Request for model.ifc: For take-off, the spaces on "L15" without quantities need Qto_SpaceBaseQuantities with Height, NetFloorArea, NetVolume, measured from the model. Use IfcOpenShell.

First a look at what the model holds.

```python
import ifcopenshell
import ifcopenshell.util.element
import ifcopenshell.util.unit

model = ifcopenshell.open("model.ifc")
print(model.schema)
for unit_type in ("LENGTHUNIT", "AREAUNIT", "VOLUMEUNIT"):
    print(unit_type, ifcopenshell.util.unit.calculate_unit_scale(model, unit_type))
storey = next(s for s in model.by_type("IfcBuildingStorey") if s.Name == "L15")
spaces = [e for e in ifcopenshell.util.element.get_decomposition(storey) if e.is_a("IfcSpace")]
for e in sorted(spaces, key=lambda e: e.id()):
    print(e.id(), e.is_a(), e.Name, list(ifcopenshell.util.element.get_psets(e, qtos_only=True)), sep=" | ")
```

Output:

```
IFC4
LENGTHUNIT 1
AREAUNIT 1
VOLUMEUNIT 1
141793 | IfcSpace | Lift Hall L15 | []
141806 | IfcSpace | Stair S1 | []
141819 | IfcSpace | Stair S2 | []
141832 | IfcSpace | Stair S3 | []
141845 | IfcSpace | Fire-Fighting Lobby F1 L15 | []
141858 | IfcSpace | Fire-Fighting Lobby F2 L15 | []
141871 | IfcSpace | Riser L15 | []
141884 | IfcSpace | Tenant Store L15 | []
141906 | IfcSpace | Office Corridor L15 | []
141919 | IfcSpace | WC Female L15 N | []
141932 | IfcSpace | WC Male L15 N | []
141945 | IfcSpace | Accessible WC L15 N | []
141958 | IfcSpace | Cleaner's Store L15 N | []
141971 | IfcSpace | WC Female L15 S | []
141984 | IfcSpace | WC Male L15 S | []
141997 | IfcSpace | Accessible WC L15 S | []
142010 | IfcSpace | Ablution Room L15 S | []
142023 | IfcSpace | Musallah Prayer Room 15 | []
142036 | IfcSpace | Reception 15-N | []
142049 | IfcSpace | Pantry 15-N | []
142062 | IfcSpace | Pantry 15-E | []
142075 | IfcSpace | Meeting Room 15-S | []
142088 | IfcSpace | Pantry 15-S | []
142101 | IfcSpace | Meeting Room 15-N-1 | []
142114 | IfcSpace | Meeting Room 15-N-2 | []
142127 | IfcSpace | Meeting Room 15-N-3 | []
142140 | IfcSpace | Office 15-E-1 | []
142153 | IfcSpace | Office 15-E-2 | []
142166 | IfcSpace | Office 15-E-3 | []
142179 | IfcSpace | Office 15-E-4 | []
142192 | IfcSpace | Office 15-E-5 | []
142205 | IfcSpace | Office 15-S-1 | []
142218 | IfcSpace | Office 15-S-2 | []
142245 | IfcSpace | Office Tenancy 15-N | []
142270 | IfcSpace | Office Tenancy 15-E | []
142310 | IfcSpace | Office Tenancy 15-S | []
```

```python
import ifcopenshell
import ifcopenshell.api.pset
import ifcopenshell.geom
import ifcopenshell.util.element
import ifcopenshell.util.shape
import ifcopenshell.util.unit

model = ifcopenshell.open("model.ifc")
unit_scale = ifcopenshell.util.unit.calculate_unit_scale(model)
area_scale = ifcopenshell.util.unit.calculate_unit_scale(model, "AREAUNIT")
volume_scale = ifcopenshell.util.unit.calculate_unit_scale(model, "VOLUMEUNIT")
settings = ifcopenshell.geom.settings()

storey = next(s for s in model.by_type("IfcBuildingStorey") if s.Name == "L15")
spaces = [e for e in ifcopenshell.util.element.get_decomposition(storey) if e.is_a("IfcSpace")]

for e in sorted(spaces, key=lambda e: e.id()):
    if ifcopenshell.util.element.get_psets(e, qtos_only=True, should_inherit=False):
        continue
    # Geometry comes back in metres, in the element's own axes.
    shape = ifcopenshell.geom.create_shape(settings, e)
    values = {
        "Height": ifcopenshell.util.shape.get_z(shape.geometry) / unit_scale,
        "NetFloorArea": ifcopenshell.util.shape.get_footprint_area(shape.geometry) / area_scale,
        "NetVolume": ifcopenshell.util.shape.get_volume(shape.geometry) / volume_scale,
    }
    qto = ifcopenshell.api.pset.add_qto(model, product=e, name="Qto_SpaceBaseQuantities")
    ifcopenshell.api.pset.edit_qto(model, qto=qto, properties=values)
    print(e.id(), {k: round(v, 3) for k, v in values.items()})

model.write("model_rev.ifc")
```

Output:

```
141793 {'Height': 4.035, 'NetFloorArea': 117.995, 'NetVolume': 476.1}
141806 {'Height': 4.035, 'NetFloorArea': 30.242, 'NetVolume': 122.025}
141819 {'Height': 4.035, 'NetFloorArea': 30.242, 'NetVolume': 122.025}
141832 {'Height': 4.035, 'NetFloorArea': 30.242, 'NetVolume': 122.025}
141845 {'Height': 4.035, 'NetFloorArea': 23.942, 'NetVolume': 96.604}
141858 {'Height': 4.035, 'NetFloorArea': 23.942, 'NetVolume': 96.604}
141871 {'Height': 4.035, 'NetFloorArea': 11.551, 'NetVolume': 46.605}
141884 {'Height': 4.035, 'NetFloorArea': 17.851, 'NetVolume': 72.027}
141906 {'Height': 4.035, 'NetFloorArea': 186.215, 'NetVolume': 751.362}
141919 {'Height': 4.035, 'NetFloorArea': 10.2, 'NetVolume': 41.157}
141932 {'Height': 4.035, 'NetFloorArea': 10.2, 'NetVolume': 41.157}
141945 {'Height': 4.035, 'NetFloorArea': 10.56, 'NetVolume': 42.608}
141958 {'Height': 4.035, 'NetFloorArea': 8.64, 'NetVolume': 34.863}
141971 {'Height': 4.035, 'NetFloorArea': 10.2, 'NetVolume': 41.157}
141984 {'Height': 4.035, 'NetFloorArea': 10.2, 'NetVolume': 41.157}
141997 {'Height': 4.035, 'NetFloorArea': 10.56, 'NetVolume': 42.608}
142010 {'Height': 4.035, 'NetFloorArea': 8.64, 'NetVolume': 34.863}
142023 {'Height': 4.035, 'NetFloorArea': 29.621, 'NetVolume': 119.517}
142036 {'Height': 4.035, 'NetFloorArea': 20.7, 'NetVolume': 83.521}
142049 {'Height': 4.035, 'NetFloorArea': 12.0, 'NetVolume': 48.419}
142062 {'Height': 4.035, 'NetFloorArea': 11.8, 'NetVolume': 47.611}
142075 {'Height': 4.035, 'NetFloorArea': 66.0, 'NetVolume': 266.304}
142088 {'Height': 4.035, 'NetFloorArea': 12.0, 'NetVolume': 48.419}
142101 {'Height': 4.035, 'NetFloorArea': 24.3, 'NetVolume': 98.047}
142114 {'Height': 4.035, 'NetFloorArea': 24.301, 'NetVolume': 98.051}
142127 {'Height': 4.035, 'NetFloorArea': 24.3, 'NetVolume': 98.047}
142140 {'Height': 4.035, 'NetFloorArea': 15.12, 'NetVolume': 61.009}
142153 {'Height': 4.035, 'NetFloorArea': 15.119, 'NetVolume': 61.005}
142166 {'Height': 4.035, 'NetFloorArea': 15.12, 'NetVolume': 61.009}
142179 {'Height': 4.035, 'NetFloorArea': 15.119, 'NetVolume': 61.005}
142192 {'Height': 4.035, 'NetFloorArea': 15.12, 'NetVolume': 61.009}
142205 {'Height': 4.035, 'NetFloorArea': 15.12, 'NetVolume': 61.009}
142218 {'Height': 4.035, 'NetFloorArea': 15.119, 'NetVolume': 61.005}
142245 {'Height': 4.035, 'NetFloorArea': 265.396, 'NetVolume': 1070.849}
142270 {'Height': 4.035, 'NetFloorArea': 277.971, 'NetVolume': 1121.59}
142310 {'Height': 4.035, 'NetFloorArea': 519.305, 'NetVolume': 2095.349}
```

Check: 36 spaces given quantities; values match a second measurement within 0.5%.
